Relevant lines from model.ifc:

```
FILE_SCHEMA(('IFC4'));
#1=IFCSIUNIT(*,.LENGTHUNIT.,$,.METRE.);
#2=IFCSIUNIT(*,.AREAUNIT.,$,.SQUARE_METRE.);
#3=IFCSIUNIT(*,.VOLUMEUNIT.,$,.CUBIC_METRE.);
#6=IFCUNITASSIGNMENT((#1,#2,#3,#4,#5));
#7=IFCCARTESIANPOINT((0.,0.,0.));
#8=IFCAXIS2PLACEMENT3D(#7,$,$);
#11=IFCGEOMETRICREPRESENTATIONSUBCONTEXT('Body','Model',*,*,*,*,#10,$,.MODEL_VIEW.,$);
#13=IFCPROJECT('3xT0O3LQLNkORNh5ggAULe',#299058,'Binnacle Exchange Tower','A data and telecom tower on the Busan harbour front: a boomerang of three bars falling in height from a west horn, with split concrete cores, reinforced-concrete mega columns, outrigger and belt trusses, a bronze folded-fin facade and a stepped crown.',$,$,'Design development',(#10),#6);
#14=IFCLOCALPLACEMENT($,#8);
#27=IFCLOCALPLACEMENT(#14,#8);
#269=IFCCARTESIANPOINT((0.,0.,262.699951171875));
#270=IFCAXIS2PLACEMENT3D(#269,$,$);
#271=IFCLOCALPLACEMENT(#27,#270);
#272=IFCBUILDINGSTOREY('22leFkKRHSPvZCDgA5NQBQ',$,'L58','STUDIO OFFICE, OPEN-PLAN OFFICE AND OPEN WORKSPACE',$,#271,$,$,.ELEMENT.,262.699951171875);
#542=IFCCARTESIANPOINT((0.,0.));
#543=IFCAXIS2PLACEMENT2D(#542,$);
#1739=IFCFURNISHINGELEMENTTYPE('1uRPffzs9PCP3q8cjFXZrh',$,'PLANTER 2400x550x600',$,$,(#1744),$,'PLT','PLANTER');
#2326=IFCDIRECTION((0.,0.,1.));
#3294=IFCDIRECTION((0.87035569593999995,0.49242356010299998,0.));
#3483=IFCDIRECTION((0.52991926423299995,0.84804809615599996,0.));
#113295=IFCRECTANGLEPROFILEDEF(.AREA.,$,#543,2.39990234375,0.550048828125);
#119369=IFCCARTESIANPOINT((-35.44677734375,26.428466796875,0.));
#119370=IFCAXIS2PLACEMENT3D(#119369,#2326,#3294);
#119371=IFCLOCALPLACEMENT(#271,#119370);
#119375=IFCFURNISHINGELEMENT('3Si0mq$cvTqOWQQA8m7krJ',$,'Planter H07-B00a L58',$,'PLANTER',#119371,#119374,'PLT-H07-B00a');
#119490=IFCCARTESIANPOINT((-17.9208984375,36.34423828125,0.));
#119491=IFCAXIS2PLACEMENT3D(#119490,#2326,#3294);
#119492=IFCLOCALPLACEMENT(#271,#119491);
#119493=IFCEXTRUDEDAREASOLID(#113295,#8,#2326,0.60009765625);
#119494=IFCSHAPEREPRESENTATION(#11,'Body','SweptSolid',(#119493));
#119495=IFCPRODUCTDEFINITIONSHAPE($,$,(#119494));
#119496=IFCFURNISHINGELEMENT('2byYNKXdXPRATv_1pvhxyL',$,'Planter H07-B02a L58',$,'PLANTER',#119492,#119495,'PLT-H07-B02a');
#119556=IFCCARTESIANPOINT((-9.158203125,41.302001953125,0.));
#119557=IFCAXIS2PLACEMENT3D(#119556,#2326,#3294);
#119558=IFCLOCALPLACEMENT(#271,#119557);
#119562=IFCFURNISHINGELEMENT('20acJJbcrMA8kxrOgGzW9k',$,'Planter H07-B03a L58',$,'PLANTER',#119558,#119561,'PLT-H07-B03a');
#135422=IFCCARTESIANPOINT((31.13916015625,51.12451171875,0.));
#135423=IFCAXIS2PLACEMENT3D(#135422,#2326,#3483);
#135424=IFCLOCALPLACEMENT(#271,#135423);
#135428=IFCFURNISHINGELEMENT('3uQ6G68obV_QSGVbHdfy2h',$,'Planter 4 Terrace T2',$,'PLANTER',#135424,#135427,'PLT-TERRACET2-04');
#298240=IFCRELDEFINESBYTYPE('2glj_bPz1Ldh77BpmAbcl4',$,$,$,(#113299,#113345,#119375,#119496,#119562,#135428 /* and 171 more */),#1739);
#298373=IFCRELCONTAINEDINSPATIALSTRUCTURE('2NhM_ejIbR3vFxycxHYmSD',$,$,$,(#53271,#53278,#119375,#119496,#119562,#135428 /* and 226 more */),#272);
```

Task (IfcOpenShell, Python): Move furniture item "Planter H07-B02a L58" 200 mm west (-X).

```python
import ifcopenshell
import ifcopenshell.api.geometry
import ifcopenshell.util.placement

model = ifcopenshell.open("model.ifc")

item = model.by_guid("2byYNKXdXPRATv_1pvhxyL")
matrix = ifcopenshell.util.placement.get_local_placement(item.ObjectPlacement)
matrix[0, 3] -= 0.2
ifcopenshell.api.geometry.edit_object_placement(model, product=item, matrix=matrix, is_si=False)

print(ifcopenshell.util.placement.get_local_placement(item.ObjectPlacement).round(3) + 0.0)

model.write("model-out.ifc")
```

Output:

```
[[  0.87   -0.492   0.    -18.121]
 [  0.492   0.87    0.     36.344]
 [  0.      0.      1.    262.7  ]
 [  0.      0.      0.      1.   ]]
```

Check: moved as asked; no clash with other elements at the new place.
